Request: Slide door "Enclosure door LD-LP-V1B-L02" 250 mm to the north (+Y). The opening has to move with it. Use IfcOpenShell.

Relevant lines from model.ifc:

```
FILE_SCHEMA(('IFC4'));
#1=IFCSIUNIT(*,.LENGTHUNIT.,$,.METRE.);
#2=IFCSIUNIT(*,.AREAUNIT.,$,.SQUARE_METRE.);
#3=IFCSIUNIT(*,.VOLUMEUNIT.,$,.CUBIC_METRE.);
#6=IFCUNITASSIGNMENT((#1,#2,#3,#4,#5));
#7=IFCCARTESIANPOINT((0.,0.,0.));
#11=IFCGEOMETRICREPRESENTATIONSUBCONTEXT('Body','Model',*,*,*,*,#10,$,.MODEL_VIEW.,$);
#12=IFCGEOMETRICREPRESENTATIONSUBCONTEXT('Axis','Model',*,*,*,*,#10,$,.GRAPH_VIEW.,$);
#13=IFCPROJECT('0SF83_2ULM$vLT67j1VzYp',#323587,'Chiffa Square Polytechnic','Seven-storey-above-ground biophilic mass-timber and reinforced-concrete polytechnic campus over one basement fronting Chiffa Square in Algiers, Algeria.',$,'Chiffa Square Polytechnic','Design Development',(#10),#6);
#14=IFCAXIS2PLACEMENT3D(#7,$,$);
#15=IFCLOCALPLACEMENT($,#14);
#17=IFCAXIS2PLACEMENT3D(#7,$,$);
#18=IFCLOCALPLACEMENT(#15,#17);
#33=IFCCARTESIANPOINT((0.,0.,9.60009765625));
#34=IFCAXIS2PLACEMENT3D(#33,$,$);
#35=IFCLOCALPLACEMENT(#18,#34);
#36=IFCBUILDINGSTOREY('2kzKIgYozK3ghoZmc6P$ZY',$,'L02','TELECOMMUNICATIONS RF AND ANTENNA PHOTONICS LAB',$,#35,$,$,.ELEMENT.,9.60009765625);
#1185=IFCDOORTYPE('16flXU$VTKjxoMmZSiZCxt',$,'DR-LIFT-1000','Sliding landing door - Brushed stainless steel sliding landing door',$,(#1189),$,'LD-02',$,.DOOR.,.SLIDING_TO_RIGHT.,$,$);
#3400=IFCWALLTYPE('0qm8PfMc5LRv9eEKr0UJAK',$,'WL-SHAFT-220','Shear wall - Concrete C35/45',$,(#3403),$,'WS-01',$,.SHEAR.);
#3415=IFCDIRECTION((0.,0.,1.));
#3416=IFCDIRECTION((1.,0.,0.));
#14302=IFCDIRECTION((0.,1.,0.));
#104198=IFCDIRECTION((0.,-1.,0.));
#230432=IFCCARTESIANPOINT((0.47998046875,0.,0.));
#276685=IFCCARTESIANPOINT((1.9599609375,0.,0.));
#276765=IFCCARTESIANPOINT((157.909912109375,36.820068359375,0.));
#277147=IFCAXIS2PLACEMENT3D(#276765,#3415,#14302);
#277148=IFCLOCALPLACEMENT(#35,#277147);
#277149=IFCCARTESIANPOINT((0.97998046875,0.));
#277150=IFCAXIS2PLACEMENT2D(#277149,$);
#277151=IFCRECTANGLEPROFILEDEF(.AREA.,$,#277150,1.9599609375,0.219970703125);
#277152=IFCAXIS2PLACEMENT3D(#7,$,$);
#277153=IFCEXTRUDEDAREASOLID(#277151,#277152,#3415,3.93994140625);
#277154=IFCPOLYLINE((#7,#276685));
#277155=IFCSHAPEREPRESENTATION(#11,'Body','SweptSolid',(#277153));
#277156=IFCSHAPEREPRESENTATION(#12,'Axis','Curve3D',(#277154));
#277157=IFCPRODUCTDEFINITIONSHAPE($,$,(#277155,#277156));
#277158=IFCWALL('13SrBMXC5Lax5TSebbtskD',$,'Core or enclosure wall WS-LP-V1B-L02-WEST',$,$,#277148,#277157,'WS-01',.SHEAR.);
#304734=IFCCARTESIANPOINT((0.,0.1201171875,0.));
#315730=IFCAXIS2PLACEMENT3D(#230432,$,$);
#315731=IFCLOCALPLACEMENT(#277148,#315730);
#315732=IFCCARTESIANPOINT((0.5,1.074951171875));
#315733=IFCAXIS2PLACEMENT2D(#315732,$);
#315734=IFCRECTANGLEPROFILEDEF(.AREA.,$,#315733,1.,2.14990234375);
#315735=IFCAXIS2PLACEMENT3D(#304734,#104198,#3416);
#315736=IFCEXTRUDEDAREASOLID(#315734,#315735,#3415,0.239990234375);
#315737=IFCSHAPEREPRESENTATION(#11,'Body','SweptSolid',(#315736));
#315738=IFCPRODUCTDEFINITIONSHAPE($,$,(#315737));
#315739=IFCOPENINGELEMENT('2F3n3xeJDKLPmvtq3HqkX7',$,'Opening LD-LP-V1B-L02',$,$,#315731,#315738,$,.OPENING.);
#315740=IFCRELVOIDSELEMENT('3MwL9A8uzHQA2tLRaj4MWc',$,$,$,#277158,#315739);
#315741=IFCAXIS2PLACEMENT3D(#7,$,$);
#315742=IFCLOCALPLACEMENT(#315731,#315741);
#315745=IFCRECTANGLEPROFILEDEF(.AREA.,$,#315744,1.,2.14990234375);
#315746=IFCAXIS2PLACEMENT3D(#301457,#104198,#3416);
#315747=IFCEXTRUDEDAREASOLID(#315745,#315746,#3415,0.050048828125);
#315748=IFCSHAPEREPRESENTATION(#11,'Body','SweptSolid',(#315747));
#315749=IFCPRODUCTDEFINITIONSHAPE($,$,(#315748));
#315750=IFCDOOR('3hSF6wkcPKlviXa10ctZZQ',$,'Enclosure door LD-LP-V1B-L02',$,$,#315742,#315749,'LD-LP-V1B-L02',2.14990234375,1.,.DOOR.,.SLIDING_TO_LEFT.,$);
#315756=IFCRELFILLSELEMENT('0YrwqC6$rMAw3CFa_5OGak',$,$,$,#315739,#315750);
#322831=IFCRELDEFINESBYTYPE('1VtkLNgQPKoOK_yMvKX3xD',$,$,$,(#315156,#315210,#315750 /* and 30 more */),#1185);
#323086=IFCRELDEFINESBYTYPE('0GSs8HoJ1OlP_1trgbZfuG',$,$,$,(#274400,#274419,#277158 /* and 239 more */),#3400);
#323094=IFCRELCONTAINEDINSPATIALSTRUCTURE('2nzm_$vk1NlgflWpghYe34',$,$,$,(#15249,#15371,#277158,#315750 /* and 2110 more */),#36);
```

```python
import ifcopenshell
import ifcopenshell.api.geometry
import ifcopenshell.util.placement
import ifcopenshell.util.unit

model = ifcopenshell.open("model.ifc")
unit_scale = ifcopenshell.util.unit.calculate_unit_scale(model)

door = model.by_id(315750)
opening = door.FillsVoids[0].RelatingOpeningElement
wall = opening.VoidsElements[0].RelatingBuildingElement

wall_matrix = ifcopenshell.util.placement.get_local_placement(wall.ObjectPlacement)
shift = wall_matrix[:3, 0] * 0.25 / unit_scale
before = ifcopenshell.util.placement.get_local_placement(door.ObjectPlacement)[:3, 3].copy()

# The door is placed relative to its opening, so it follows when the opening moves.
matrix = ifcopenshell.util.placement.get_local_placement(opening.ObjectPlacement)
matrix[:3, 3] += shift
ifcopenshell.api.geometry.edit_object_placement(
    model, product=opening, matrix=matrix, is_si=False, should_transform_children=True
)

after = ifcopenshell.util.placement.get_local_placement(door.ObjectPlacement)[:3, 3]
print("door moved by", (after - before).round(3) + 0.0)

model.write("model_updated.ifc")
```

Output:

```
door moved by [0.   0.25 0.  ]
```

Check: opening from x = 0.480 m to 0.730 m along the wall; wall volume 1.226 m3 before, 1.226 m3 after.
